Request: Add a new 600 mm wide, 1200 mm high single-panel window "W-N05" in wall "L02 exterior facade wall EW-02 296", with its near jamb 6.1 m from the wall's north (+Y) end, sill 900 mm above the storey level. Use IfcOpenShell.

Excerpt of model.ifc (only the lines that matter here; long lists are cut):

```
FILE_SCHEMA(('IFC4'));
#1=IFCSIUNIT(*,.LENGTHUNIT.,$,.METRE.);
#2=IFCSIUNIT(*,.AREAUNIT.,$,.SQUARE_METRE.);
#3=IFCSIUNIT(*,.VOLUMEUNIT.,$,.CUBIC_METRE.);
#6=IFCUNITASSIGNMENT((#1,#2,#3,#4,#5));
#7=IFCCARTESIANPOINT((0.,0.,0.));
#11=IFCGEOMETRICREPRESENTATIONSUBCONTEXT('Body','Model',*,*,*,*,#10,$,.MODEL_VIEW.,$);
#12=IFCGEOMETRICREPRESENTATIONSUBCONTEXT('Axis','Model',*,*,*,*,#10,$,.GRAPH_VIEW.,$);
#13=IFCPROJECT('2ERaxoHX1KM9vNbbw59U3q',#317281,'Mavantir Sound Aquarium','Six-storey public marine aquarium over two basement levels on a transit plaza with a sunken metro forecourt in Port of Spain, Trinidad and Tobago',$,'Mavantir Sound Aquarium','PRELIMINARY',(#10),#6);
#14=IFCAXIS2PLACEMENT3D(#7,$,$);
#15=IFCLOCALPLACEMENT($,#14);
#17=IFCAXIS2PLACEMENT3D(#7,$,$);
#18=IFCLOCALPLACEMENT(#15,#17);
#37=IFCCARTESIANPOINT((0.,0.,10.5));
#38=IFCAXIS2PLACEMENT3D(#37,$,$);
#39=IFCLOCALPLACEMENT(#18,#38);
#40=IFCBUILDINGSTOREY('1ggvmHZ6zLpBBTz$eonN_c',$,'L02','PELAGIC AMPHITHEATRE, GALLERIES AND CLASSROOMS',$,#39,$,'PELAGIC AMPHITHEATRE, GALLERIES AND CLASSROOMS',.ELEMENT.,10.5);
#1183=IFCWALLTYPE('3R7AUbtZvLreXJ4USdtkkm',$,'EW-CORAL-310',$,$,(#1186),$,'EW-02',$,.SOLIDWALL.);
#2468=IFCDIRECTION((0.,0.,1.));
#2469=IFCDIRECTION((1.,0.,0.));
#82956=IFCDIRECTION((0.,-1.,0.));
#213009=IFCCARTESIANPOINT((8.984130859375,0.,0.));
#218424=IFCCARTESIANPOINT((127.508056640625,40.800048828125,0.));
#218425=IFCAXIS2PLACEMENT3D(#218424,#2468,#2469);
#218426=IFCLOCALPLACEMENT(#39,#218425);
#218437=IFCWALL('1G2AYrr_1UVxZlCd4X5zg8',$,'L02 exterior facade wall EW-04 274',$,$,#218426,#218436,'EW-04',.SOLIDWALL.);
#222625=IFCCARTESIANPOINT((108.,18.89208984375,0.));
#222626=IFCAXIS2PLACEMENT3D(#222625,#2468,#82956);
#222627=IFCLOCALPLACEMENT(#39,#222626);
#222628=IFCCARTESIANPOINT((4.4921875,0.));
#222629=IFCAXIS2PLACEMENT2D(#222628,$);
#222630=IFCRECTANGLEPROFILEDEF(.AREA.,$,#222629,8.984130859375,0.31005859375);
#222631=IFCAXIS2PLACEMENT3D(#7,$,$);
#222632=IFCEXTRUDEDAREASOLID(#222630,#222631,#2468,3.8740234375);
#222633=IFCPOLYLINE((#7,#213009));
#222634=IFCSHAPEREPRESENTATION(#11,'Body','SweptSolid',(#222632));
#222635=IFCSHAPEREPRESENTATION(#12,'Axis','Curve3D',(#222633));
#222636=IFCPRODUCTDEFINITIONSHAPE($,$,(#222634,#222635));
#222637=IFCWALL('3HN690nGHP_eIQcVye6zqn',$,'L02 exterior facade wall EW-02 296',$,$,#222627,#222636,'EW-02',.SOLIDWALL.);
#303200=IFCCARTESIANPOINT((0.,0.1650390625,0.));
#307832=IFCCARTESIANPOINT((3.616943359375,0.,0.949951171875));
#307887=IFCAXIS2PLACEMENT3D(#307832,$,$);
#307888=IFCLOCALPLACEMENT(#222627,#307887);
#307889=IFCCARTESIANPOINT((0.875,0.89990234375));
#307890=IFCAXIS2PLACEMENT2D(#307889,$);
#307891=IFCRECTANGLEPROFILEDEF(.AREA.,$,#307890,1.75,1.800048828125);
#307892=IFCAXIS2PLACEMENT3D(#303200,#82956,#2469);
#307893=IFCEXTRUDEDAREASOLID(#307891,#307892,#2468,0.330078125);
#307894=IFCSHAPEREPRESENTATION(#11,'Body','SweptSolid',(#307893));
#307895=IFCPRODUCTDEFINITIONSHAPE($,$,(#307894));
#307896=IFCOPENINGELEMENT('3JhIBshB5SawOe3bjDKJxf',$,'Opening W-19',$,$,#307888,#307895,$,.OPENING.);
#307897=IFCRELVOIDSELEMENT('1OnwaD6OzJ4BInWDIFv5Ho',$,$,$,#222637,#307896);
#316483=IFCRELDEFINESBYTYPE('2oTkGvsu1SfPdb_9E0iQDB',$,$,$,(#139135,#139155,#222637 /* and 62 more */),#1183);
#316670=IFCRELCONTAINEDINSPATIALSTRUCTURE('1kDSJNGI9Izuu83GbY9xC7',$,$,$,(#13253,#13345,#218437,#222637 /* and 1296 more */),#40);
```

```python
import numpy as np
import ifcopenshell
import ifcopenshell.api.feature
import ifcopenshell.api.geometry
import ifcopenshell.api.root
import ifcopenshell.api.spatial
import ifcopenshell.geom
import ifcopenshell.util.element
import ifcopenshell.util.placement
import ifcopenshell.util.representation
import ifcopenshell.util.shape
import ifcopenshell.util.unit

model = ifcopenshell.open("model.ifc")
unit_scale = ifcopenshell.util.unit.calculate_unit_scale(model)
settings = ifcopenshell.geom.settings()


def volume(element):
    """Net volume in cubic metres, openings subtracted."""
    shape = ifcopenshell.geom.create_shape(settings, element)
    return ifcopenshell.util.shape.get_volume(shape.geometry)


wall = model.by_guid("3HN690nGHP_eIQcVye6zqn")
storey = ifcopenshell.util.element.get_container(wall, ifc_class="IfcBuildingStorey")
context = ifcopenshell.util.representation.get_context(model, "Model", "Body", "MODEL_VIEW")
before = volume(wall)

width, height, from_end, sill = 0.6, 1.2, 6.1, 0.9  # metres

# The wall runs along its own X axis, and the end named is its -X end.
wall_shape = ifcopenshell.geom.create_shape(settings, wall)
x, y, z = ifcopenshell.util.shape.get_vertices(wall_shape.geometry).T
start = x.min() + from_end
face, thickness = float(y.min()), float(y.max() - y.min())
wall_matrix = ifcopenshell.util.placement.get_local_placement(wall.ObjectPlacement)
level = ifcopenshell.util.placement.get_local_placement(storey.ObjectPlacement)[2, 3]


def in_wall(x, y):
    """Placement at x, y metres in the wall's axes, at sill height."""
    matrix = wall_matrix.copy()
    matrix[:, 3] = wall_matrix @ np.array([x / unit_scale, y / unit_scale, 0.0, 1.0])
    matrix[2, 3] = level + sill / unit_scale
    return matrix


# Opening: a box that overshoots both wall faces by 50 mm.
opening = ifcopenshell.api.root.create_entity(model, ifc_class="IfcOpeningElement", predefined_type="OPENING")
box = ifcopenshell.api.geometry.add_wall_representation(
    model, context=context, length=width, height=height, thickness=thickness + 0.1
)
ifcopenshell.api.geometry.assign_representation(model, product=opening, representation=box)
ifcopenshell.api.geometry.edit_object_placement(model, product=opening, matrix=in_wall(start, face - 0.05), is_si=False)
ifcopenshell.api.feature.add_feature(model, feature=opening, element=wall)

window = ifcopenshell.api.root.create_entity(model, ifc_class="IfcWindow", name="W-N05", predefined_type="WINDOW")
window.OverallWidth, window.OverallHeight = width / unit_scale, height / unit_scale
window.PartitioningType = "SINGLE_PANEL"
body = ifcopenshell.api.geometry.add_window_representation(
    model,
    context=context,
    overall_width=window.OverallWidth,
    overall_height=window.OverallHeight,
    partition_type="SINGLE_PANEL",
)
ifcopenshell.api.geometry.assign_representation(model, product=window, representation=body)
ifcopenshell.api.spatial.assign_container(model, products=[window], relating_structure=storey)
ifcopenshell.api.feature.add_filling(model, opening=opening, element=window)

# Centre the window in the wall's thickness.
ifcopenshell.api.geometry.edit_object_placement(model, product=window, matrix=in_wall(start, face), is_si=False)
window_shape = ifcopenshell.geom.create_shape(settings, window)
depth = ifcopenshell.util.shape.get_vertices(window_shape.geometry)[:, 1]
offset = face + thickness / 2 - (depth.min() + depth.max()) / 2
ifcopenshell.api.geometry.edit_object_placement(model, product=window, matrix=in_wall(start, offset), is_si=False)

after = volume(wall)

print(f"wall volume {before:.3f} -> {after:.3f} m3")

model.write("model_rev.ifc")
```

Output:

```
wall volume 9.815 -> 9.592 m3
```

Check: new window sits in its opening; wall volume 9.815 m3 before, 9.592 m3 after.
